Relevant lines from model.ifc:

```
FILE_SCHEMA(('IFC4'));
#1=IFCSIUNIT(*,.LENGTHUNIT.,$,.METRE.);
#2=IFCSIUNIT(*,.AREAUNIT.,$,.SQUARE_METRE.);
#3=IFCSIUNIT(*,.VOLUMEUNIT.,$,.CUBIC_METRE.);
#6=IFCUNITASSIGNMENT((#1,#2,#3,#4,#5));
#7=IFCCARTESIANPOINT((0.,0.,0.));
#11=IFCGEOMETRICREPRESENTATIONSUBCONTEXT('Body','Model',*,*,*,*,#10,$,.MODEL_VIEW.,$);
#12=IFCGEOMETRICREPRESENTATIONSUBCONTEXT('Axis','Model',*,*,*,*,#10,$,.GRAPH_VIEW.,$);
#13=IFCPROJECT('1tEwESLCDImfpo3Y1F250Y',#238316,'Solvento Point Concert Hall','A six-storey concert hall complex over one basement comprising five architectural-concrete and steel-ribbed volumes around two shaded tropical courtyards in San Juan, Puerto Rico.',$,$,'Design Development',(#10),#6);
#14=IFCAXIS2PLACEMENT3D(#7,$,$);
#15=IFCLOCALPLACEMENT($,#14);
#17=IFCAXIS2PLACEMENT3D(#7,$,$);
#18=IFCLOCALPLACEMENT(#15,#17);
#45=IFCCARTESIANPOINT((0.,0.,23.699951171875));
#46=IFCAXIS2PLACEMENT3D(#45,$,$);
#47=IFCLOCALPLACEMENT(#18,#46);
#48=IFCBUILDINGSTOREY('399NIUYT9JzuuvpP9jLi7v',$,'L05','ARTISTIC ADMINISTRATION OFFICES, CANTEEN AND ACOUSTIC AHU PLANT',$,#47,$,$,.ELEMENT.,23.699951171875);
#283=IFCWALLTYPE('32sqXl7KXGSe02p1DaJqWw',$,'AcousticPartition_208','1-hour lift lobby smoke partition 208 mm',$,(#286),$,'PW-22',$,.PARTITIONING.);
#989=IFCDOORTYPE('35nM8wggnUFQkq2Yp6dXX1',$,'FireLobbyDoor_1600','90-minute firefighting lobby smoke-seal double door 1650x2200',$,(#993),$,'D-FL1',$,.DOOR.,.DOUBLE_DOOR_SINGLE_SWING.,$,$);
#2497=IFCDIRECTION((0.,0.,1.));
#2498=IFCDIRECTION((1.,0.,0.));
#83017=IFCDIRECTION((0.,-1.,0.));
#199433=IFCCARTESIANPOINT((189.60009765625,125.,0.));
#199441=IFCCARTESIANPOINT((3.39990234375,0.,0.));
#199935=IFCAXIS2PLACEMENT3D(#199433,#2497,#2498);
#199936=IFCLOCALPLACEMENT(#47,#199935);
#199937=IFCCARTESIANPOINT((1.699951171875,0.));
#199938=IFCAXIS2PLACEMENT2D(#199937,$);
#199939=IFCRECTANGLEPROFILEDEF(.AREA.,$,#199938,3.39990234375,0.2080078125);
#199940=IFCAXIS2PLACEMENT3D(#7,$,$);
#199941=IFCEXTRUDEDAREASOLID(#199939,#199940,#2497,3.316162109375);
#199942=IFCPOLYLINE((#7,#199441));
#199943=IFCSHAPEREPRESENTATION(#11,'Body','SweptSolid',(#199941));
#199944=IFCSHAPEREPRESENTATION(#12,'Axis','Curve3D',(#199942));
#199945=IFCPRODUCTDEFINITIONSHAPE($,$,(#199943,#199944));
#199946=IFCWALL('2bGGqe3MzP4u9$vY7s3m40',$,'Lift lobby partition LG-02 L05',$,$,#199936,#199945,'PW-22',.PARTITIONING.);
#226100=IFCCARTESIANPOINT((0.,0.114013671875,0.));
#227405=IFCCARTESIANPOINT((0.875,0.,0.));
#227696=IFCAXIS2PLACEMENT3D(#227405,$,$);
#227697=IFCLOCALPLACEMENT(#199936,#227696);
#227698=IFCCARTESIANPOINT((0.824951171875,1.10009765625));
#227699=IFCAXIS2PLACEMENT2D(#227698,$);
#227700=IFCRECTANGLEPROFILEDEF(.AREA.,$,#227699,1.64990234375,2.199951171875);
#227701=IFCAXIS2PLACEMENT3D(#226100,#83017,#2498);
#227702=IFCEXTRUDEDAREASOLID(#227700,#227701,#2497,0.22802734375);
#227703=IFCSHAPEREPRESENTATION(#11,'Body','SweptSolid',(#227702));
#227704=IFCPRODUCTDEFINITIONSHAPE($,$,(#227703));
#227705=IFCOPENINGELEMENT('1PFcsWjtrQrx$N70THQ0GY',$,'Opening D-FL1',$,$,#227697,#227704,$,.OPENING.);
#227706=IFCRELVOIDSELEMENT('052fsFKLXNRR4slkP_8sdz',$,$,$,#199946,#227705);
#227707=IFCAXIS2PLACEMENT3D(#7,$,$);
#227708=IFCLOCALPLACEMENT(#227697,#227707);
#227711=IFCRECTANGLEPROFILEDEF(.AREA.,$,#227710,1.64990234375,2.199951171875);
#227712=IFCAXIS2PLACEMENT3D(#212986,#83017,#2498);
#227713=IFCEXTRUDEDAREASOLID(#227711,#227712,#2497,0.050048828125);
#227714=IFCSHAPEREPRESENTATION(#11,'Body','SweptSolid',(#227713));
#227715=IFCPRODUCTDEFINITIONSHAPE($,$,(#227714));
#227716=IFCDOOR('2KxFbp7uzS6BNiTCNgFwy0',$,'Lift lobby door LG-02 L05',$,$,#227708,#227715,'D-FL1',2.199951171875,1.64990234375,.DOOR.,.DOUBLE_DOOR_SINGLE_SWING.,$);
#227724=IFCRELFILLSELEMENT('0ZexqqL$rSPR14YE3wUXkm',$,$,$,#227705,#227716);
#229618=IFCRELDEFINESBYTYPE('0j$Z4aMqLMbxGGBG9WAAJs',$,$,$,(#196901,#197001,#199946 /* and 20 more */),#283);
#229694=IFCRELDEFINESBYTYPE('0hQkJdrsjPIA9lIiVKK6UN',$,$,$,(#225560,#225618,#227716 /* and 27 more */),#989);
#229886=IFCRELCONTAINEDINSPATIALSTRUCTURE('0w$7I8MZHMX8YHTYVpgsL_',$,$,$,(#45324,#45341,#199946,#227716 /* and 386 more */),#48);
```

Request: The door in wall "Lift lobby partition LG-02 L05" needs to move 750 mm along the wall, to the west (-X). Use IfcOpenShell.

```python
import ifcopenshell
import ifcopenshell.api.geometry
import ifcopenshell.util.placement
import ifcopenshell.util.unit

model = ifcopenshell.open("model.ifc")
unit_scale = ifcopenshell.util.unit.calculate_unit_scale(model)

door = model.by_guid("2KxFbp7uzS6BNiTCNgFwy0")
opening = door.FillsVoids[0].RelatingOpeningElement
wall = opening.VoidsElements[0].RelatingBuildingElement

wall_matrix = ifcopenshell.util.placement.get_local_placement(wall.ObjectPlacement)
shift = wall_matrix[:3, 0] * -0.75 / unit_scale
before = ifcopenshell.util.placement.get_local_placement(door.ObjectPlacement)[:3, 3].copy()

# The door is placed relative to its opening, so it follows when the opening moves.
matrix = ifcopenshell.util.placement.get_local_placement(opening.ObjectPlacement)
matrix[:3, 3] += shift
ifcopenshell.api.geometry.edit_object_placement(
    model, product=opening, matrix=matrix, is_si=False, should_transform_children=True
)

after = ifcopenshell.util.placement.get_local_placement(door.ObjectPlacement)[:3, 3]
print("door moved by", (after - before).round(3) + 0.0)

model.write("model-out.ifc")
```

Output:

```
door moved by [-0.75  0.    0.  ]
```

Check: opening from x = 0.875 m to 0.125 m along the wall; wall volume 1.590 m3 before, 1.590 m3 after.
